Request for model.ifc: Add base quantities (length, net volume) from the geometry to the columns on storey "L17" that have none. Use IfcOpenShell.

First a look at what the model holds.

```python
import ifcopenshell
import ifcopenshell.util.element
import ifcopenshell.util.unit

model = ifcopenshell.open("model.ifc")
print(model.schema)
for unit_type in ("LENGTHUNIT", "AREAUNIT", "VOLUMEUNIT"):
    print(unit_type, ifcopenshell.util.unit.calculate_unit_scale(model, unit_type))
storey = next(s for s in model.by_type("IfcBuildingStorey") if s.Name == "L17")
columns = [e for e in ifcopenshell.util.element.get_decomposition(storey) if e.is_a("IfcColumn")]
for e in sorted(columns, key=lambda e: e.id()):
    print(e.id(), e.is_a(), e.Name, list(ifcopenshell.util.element.get_psets(e, qtos_only=True)), sep=" | ")
```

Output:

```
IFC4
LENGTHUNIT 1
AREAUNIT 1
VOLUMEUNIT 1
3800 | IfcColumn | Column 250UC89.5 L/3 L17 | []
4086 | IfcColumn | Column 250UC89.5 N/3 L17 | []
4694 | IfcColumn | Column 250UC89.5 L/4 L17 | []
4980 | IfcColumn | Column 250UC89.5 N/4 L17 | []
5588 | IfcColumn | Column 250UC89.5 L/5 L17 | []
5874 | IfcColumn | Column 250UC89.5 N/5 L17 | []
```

```python
import ifcopenshell
import ifcopenshell.api.pset
import ifcopenshell.geom
import ifcopenshell.util.element
import ifcopenshell.util.shape
import ifcopenshell.util.unit

model = ifcopenshell.open("model.ifc")
unit_scale = ifcopenshell.util.unit.calculate_unit_scale(model)
volume_scale = ifcopenshell.util.unit.calculate_unit_scale(model, "VOLUMEUNIT")
settings = ifcopenshell.geom.settings()

storey = next(s for s in model.by_type("IfcBuildingStorey") if s.Name == "L17")
columns = [e for e in ifcopenshell.util.element.get_decomposition(storey) if e.is_a("IfcColumn")]

for e in sorted(columns, key=lambda e: e.id()):
    if ifcopenshell.util.element.get_psets(e, qtos_only=True, should_inherit=False):
        continue
    # Geometry comes back in metres, in the element's own axes.
    shape = ifcopenshell.geom.create_shape(settings, e)
    values = {
        "Length": ifcopenshell.util.shape.get_z(shape.geometry) / unit_scale,
        "NetVolume": ifcopenshell.util.shape.get_volume(shape.geometry) / volume_scale,
    }
    qto = ifcopenshell.api.pset.add_qto(model, product=e, name="Qto_ColumnBaseQuantities")
    ifcopenshell.api.pset.edit_qto(model, qto=qto, properties=values)
    print(e.id(), {k: round(v, 3) for k, v in values.items()})

model.write("model_edited.ifc")
```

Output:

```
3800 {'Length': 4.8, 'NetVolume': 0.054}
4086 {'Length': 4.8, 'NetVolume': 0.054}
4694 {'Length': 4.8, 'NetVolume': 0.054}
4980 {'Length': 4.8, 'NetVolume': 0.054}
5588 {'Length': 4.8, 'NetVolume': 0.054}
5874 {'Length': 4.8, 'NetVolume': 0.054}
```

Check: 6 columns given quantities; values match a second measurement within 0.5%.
